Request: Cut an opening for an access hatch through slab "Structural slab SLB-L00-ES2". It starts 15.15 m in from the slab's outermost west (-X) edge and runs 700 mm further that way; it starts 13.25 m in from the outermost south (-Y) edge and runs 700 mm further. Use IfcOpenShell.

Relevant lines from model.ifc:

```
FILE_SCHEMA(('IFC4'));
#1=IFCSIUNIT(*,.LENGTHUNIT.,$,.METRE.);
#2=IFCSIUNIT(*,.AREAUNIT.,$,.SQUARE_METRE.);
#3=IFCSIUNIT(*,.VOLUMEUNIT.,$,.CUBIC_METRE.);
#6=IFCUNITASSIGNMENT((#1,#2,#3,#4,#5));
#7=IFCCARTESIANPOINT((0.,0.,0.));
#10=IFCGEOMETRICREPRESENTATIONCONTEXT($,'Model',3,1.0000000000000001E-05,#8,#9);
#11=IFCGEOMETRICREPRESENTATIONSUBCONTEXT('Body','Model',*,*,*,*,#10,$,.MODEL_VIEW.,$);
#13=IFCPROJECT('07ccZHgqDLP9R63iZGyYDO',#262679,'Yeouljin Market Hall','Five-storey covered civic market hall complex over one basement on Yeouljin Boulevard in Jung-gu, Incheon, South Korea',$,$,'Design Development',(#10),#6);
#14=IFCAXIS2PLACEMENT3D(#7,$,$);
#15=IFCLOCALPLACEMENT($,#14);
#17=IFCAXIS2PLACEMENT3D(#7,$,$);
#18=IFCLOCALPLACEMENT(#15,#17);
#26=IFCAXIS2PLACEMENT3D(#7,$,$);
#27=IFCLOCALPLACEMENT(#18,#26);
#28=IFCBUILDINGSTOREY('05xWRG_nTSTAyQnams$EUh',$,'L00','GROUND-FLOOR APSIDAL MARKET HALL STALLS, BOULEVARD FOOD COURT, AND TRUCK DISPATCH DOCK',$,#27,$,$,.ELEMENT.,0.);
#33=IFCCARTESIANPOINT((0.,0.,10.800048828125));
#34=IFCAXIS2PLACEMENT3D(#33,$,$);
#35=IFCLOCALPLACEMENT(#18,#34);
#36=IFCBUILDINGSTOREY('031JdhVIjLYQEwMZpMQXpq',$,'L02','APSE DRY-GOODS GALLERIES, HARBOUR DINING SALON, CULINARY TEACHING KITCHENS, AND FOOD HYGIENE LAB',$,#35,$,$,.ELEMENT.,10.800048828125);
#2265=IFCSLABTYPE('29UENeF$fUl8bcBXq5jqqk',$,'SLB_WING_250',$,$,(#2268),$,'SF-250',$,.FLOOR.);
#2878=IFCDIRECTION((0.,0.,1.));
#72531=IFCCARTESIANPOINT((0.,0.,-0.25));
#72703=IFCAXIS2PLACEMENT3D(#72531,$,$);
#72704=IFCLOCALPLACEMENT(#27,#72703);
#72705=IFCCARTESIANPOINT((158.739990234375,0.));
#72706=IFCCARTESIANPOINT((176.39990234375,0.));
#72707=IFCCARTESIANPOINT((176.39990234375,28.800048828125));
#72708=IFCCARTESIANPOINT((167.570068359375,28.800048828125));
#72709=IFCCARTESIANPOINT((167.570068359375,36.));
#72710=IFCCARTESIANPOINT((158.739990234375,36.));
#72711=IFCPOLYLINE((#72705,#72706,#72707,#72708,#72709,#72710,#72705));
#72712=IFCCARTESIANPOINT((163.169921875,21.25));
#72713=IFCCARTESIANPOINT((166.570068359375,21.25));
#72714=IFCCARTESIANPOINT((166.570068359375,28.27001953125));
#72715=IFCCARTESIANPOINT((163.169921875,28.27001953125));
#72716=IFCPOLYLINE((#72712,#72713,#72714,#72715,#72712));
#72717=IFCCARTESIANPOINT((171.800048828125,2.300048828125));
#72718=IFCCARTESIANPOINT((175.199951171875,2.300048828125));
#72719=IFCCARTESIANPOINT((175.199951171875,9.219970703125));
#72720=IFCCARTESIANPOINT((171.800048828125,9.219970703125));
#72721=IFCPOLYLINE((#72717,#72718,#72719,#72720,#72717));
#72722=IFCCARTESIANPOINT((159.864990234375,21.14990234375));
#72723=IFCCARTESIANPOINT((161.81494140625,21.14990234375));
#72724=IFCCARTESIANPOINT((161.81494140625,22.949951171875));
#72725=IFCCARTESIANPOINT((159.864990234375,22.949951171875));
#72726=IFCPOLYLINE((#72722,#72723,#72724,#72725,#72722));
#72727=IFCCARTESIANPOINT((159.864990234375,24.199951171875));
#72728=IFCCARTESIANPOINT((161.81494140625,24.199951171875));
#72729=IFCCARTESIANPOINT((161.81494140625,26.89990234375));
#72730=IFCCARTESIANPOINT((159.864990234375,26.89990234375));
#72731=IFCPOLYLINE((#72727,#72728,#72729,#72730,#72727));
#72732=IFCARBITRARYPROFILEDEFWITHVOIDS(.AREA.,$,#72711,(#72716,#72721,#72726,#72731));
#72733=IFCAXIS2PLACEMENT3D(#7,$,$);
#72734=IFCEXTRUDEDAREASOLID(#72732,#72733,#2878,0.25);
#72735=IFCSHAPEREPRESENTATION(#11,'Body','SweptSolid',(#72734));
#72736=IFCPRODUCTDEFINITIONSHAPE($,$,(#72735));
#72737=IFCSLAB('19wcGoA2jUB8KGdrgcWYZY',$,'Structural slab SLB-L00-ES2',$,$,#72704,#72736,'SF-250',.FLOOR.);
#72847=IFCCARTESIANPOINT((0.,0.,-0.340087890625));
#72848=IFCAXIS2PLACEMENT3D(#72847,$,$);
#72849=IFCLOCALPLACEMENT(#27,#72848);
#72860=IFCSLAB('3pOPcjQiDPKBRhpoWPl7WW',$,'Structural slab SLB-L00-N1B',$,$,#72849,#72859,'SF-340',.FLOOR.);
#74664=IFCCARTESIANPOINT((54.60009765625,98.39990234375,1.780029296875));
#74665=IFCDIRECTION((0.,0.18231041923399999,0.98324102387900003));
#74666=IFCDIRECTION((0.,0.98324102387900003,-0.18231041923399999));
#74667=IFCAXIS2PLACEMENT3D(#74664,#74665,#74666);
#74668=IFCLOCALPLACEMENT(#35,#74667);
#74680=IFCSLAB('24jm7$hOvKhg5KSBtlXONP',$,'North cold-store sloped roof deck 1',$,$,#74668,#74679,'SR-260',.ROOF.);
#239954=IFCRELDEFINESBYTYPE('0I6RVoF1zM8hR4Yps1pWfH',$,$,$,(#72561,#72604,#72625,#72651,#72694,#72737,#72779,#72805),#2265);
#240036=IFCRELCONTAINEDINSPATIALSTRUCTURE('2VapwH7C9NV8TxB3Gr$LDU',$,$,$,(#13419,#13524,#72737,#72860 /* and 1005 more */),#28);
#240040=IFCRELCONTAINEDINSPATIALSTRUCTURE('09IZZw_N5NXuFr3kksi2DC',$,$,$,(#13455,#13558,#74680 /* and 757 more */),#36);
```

```python
import numpy as np
import ifcopenshell
import ifcopenshell.api.feature
import ifcopenshell.api.geometry
import ifcopenshell.api.root
import ifcopenshell.geom
import ifcopenshell.util.placement
import ifcopenshell.util.representation
import ifcopenshell.util.shape
import ifcopenshell.util.unit

model = ifcopenshell.open("model.ifc")
unit_scale = ifcopenshell.util.unit.calculate_unit_scale(model)
settings = ifcopenshell.geom.settings()


def volume(element):
    """Net volume in cubic metres, openings subtracted."""
    shape = ifcopenshell.geom.create_shape(settings, element)
    return ifcopenshell.util.shape.get_volume(shape.geometry)


slab = model.by_guid("19wcGoA2jUB8KGdrgcWYZY")
before = volume(slab)

# Extent in the slab's own axes, in metres. The edges named are its -X and -Y sides.
slab_shape = ifcopenshell.geom.create_shape(settings, slab)
vertices = ifcopenshell.util.shape.get_vertices(slab_shape.geometry)
x_min, y_min, bottom = vertices.min(axis=0)
top = vertices[:, 2].max()

opening = ifcopenshell.api.root.create_entity(model, ifc_class="IfcOpeningElement", name="Access hatch opening", predefined_type="OPENING")
context = ifcopenshell.util.representation.get_context(model, "Model", "Body", "MODEL_VIEW")
width, depth = 0.7, 0.7
outline = [(0.0, 0.0), (width, 0.0), (width, depth), (0.0, depth), (0.0, 0.0)]
# Overshoot both faces by 50 mm so the cut is clean.
shape = ifcopenshell.api.geometry.add_slab_representation(
    model, context=context, depth=top - bottom + 0.1, polyline=outline
)
ifcopenshell.api.geometry.assign_representation(model, product=opening, representation=shape)

matrix = ifcopenshell.util.placement.get_local_placement(slab.ObjectPlacement)
matrix[:, 3] = matrix @ np.append(np.array([x_min + 15.15, y_min + 13.25, bottom - 0.05]) / unit_scale, 1.0)
ifcopenshell.api.geometry.edit_object_placement(model, product=opening, matrix=matrix, is_si=False)
ifcopenshell.api.feature.add_feature(model, feature=opening, element=slab)

after = volume(slab)

print(f"slab volume {before:.3f} -> {after:.3f} m3")

model.write("model_updated.ifc")
```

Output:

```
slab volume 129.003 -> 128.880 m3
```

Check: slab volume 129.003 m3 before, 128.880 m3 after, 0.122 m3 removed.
